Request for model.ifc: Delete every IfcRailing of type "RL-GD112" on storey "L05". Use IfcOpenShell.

First a look at what the model holds.

```python
import ifcopenshell
import ifcopenshell.util.element

model = ifcopenshell.open("model.ifc")
print(model.schema)
storey = next(s for s in model.by_type("IfcBuildingStorey") if s.Name == "L05")
railings = [e for e in ifcopenshell.util.element.get_decomposition(storey) if e.is_a("IfcRailing")]
seen = {}
for e in railings:
    element_type = ifcopenshell.util.element.get_type(e)
    name = element_type.Name if element_type not in (None, e) else None
    seen[name] = seen.get(name, 0) + 1
for name, count in sorted(seen.items(), key=str):
    print(count, "x", name)
```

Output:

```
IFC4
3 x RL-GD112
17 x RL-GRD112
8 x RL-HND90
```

```python
import ifcopenshell
import ifcopenshell.api.root
import ifcopenshell.util.element

model = ifcopenshell.open("model.ifc")

storey = next(s for s in model.by_type("IfcBuildingStorey") if s.Name == "L05")
railings = [e for e in ifcopenshell.util.element.get_decomposition(storey) if e.is_a("IfcRailing")]
targets = [e for e in railings if (t := ifcopenshell.util.element.get_type(e)) not in (None, e) and t.Name == "RL-GD112"]

for e in targets:
    ifcopenshell.api.root.remove_product(model, product=e)
print(len(targets), "removed")

model.write("model-out.ifc")
```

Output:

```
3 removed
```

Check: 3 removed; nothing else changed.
